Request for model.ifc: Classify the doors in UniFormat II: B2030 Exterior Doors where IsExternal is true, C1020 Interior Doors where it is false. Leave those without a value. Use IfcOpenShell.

First a look at what the model holds.

```python
import ifcopenshell
import ifcopenshell.util.element

model = ifcopenshell.open("model.ifc")
print(model.schema)
print("classifications:", [c.Name for c in model.by_type("IfcClassification")])
values = [ifcopenshell.util.element.get_pset(e, "Pset_DoorCommon", "IsExternal") for e in model.by_type("IfcDoor")]
for value in (True, False, None):
    print("IsExternal", value, values.count(value))
```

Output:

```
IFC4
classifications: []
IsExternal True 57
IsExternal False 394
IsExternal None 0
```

```python
import ifcopenshell
import ifcopenshell.api.classification
import ifcopenshell.util.element

model = ifcopenshell.open("model.ifc")

system = ifcopenshell.api.classification.add_classification(model, classification="UniFormat II")

doors = model.by_type("IfcDoor")
external = {e: ifcopenshell.util.element.get_pset(e, "Pset_DoorCommon", "IsExternal") for e in doors}
for flag, code, name in ((True, "B2030", "Exterior Doors"), (False, "C1020", "Interior Doors")):
    products = [e for e in doors if external[e] is flag]
    ifcopenshell.api.classification.add_reference(
        model, products=products, classification=system, identification=code, name=name
    )
    print(code, len(products))

model.write("model_edited.ifc")
```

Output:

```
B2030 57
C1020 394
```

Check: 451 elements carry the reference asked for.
